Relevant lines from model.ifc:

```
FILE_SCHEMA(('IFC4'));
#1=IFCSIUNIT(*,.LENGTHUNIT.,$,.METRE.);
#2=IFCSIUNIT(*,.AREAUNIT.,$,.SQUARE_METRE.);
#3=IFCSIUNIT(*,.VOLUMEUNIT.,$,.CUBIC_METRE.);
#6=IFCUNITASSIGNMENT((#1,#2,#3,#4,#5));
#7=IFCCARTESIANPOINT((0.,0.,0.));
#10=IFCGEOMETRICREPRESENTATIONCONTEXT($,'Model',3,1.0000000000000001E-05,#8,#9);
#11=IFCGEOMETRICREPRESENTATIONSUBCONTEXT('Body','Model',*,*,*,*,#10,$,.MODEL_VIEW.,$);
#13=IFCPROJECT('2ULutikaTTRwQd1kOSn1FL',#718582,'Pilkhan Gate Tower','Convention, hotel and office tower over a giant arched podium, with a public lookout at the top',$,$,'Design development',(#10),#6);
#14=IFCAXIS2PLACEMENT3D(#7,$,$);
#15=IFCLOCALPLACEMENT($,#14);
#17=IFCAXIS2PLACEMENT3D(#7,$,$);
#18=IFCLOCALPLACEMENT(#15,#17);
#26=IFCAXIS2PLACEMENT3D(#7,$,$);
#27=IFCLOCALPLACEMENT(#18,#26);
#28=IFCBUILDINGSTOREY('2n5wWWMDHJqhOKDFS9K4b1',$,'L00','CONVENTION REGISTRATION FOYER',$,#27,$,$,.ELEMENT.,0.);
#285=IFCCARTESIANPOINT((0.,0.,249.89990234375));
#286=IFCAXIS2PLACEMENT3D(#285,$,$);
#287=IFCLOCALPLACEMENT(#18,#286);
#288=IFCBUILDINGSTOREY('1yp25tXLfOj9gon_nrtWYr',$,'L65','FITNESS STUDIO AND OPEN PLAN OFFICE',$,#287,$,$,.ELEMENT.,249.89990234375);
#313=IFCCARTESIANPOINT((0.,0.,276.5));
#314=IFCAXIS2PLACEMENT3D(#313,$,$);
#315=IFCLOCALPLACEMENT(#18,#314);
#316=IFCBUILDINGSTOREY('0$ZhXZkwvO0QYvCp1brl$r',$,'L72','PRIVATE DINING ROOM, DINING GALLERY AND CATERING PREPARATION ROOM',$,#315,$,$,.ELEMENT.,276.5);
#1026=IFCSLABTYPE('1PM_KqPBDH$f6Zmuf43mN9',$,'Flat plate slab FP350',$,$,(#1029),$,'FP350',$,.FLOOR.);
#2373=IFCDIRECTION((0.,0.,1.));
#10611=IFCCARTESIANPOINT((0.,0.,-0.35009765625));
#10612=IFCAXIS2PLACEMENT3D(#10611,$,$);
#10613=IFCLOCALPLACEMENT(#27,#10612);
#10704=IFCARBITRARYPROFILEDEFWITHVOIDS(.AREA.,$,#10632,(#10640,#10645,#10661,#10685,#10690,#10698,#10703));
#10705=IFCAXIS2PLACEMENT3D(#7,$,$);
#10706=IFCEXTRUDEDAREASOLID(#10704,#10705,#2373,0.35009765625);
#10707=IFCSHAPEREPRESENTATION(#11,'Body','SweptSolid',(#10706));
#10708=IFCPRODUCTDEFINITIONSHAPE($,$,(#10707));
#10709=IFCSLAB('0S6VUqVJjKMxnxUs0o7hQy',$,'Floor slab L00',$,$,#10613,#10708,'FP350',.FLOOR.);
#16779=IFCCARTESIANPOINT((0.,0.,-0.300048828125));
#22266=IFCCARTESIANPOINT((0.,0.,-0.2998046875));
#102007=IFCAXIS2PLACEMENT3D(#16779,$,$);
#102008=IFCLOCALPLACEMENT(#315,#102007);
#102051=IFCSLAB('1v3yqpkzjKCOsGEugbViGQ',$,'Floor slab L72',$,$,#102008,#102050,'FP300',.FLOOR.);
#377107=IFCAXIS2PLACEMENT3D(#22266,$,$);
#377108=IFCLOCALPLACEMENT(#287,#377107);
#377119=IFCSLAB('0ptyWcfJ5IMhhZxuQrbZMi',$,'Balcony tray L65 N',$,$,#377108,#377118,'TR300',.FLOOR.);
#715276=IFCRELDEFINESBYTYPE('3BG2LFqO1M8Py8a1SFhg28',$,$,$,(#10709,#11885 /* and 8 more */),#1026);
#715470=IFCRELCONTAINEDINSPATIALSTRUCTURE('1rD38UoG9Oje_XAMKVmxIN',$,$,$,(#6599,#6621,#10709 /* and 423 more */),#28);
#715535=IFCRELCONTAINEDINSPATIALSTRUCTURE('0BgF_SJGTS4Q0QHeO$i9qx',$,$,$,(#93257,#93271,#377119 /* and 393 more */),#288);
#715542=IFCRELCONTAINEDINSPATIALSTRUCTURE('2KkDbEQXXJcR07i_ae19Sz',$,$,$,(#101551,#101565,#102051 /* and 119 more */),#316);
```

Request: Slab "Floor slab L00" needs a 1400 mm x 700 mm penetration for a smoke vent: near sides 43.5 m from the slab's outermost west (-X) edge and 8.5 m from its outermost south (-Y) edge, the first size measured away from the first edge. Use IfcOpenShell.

```python
import numpy as np
import ifcopenshell
import ifcopenshell.api.feature
import ifcopenshell.api.geometry
import ifcopenshell.api.root
import ifcopenshell.geom
import ifcopenshell.util.placement
import ifcopenshell.util.representation
import ifcopenshell.util.shape
import ifcopenshell.util.unit

model = ifcopenshell.open("model.ifc")
unit_scale = ifcopenshell.util.unit.calculate_unit_scale(model)
settings = ifcopenshell.geom.settings()


def volume(element):
    """Net volume in cubic metres, openings subtracted."""
    shape = ifcopenshell.geom.create_shape(settings, element)
    return ifcopenshell.util.shape.get_volume(shape.geometry)


slab = model.by_guid("0S6VUqVJjKMxnxUs0o7hQy")
before = volume(slab)

# Extent in the slab's own axes, in metres. The edges named are its -X and -Y sides.
slab_shape = ifcopenshell.geom.create_shape(settings, slab)
vertices = ifcopenshell.util.shape.get_vertices(slab_shape.geometry)
x_min, y_min, bottom = vertices.min(axis=0)
top = vertices[:, 2].max()

opening = ifcopenshell.api.root.create_entity(model, ifc_class="IfcOpeningElement", name="Smoke vent opening", predefined_type="OPENING")
context = ifcopenshell.util.representation.get_context(model, "Model", "Body", "MODEL_VIEW")
width, depth = 1.4, 0.7
outline = [(0.0, 0.0), (width, 0.0), (width, depth), (0.0, depth), (0.0, 0.0)]
# Overshoot both faces by 50 mm so the cut is clean.
shape = ifcopenshell.api.geometry.add_slab_representation(
    model, context=context, depth=top - bottom + 0.1, polyline=outline
)
ifcopenshell.api.geometry.assign_representation(model, product=opening, representation=shape)

matrix = ifcopenshell.util.placement.get_local_placement(slab.ObjectPlacement)
matrix[:, 3] = matrix @ np.append(np.array([x_min + 43.5, y_min + 8.5, bottom - 0.05]) / unit_scale, 1.0)
ifcopenshell.api.geometry.edit_object_placement(model, product=opening, matrix=matrix, is_si=False)
ifcopenshell.api.feature.add_feature(model, feature=opening, element=slab)

after = volume(slab)

print(f"slab volume {before:.3f} -> {after:.3f} m3")

model.write("model-out.ifc")
```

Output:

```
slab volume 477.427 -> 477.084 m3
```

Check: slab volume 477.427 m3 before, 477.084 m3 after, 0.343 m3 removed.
